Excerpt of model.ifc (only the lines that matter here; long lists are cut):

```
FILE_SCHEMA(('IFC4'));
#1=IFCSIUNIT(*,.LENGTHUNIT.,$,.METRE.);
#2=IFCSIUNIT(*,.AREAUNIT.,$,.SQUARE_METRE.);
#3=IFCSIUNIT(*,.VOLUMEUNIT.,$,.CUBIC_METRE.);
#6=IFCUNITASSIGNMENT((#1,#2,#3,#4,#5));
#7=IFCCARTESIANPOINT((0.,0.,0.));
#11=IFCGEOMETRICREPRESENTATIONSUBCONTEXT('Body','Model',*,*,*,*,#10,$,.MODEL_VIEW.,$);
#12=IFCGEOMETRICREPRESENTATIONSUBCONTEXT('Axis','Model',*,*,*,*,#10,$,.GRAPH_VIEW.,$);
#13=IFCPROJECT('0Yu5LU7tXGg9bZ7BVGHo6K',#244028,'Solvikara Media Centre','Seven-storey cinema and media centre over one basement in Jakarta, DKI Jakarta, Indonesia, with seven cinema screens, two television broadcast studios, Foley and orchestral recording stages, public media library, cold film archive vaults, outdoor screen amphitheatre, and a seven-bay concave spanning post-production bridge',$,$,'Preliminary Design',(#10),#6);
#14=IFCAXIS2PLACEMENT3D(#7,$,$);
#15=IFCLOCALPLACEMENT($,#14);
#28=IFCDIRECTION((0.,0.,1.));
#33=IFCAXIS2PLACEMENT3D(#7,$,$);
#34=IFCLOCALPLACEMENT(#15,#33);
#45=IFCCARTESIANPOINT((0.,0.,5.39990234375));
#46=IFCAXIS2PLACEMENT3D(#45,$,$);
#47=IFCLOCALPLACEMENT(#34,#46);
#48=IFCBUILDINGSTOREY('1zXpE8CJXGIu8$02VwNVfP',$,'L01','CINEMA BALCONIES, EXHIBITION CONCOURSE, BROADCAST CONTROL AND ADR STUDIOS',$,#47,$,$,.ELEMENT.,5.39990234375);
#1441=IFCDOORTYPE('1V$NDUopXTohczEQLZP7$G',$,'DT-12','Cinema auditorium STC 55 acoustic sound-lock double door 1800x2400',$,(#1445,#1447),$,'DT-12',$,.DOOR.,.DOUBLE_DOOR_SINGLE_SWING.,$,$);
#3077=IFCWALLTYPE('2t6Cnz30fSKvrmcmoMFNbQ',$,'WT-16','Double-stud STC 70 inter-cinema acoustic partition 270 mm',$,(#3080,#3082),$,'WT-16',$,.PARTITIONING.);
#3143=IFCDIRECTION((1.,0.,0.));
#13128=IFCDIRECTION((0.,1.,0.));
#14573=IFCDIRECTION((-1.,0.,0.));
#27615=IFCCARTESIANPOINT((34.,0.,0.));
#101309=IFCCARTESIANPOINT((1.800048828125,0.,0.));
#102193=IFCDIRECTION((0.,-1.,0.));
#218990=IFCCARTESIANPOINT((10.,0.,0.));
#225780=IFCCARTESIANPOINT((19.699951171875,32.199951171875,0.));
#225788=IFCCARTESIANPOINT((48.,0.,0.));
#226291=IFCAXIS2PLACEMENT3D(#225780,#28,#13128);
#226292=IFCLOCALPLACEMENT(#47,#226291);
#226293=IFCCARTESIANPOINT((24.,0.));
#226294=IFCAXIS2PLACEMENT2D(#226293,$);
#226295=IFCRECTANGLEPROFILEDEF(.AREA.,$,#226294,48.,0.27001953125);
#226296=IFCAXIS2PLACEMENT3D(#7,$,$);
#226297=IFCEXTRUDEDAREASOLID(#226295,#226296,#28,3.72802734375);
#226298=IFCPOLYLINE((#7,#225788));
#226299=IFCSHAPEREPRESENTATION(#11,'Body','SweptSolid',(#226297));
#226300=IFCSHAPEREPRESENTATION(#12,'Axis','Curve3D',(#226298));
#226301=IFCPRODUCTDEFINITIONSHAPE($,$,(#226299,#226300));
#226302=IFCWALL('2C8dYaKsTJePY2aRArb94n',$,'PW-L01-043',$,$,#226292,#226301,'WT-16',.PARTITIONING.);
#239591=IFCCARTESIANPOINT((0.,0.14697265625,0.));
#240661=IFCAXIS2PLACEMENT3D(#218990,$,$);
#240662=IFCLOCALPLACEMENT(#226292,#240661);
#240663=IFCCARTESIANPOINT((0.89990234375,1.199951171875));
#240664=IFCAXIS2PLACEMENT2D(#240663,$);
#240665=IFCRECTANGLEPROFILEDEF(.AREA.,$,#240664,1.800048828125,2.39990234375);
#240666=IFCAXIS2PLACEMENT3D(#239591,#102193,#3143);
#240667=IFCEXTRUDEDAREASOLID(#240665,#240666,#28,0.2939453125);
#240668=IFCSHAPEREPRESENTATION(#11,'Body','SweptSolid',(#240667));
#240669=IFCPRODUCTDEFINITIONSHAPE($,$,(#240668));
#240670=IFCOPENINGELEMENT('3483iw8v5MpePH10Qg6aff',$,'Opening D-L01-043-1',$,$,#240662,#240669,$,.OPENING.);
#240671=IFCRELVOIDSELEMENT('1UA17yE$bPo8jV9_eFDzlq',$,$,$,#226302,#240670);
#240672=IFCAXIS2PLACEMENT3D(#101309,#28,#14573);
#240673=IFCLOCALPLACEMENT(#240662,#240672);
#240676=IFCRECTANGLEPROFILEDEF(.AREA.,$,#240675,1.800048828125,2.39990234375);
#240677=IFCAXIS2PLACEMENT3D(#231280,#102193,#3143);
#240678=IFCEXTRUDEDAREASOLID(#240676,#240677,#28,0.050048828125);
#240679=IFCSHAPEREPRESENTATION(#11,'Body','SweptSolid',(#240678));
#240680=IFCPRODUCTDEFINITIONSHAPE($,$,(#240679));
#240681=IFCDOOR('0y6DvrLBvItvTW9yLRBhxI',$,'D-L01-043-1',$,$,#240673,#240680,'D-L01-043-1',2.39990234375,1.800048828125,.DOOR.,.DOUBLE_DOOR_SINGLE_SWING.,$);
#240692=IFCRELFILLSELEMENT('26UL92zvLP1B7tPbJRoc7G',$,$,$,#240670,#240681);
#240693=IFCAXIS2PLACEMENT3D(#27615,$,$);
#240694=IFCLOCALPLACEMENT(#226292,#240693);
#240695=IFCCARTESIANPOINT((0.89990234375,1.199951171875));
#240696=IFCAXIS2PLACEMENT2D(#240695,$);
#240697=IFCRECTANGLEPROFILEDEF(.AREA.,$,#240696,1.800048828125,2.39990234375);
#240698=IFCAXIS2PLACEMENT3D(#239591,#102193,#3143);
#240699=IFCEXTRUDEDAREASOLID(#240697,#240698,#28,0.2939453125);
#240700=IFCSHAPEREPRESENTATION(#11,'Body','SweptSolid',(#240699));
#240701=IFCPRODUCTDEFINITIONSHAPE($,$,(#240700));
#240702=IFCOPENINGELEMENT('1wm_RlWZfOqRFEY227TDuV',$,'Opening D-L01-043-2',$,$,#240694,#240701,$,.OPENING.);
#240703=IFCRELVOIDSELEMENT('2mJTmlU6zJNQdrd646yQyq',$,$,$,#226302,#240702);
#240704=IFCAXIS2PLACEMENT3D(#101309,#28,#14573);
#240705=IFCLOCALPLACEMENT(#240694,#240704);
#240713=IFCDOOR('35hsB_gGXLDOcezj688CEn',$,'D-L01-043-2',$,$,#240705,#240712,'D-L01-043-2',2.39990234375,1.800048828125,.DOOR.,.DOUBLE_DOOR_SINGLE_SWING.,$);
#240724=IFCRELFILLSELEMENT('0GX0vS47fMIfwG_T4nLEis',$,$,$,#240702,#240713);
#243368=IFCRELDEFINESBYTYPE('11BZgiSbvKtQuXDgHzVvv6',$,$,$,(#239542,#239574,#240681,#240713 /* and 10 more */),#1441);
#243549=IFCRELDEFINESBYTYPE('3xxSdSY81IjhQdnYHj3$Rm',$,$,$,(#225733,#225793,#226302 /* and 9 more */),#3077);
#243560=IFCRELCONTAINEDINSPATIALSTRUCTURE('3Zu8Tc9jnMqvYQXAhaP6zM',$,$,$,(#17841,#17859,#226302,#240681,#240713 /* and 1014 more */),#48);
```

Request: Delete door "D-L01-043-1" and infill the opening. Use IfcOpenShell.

```python
import ifcopenshell
import ifcopenshell.api.feature
import ifcopenshell.api.root
import ifcopenshell.geom
import ifcopenshell.util.shape

model = ifcopenshell.open("model.ifc")
settings = ifcopenshell.geom.settings()


def volume(element):
    """Net volume in cubic metres, openings subtracted."""
    shape = ifcopenshell.geom.create_shape(settings, element)
    return ifcopenshell.util.shape.get_volume(shape.geometry)


door = model.by_id(240681)
opening = door.FillsVoids[0].RelatingOpeningElement
wall = opening.VoidsElements[0].RelatingBuildingElement
before = volume(wall)

ifcopenshell.api.root.remove_product(model, product=door)
ifcopenshell.api.feature.remove_feature(model, feature=opening)

after = volume(wall)

print(f"wall volume {before:.3f} -> {after:.3f} m3")

model.write("model_v2.ifc")
```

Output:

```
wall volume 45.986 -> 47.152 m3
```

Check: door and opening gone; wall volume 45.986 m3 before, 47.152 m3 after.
